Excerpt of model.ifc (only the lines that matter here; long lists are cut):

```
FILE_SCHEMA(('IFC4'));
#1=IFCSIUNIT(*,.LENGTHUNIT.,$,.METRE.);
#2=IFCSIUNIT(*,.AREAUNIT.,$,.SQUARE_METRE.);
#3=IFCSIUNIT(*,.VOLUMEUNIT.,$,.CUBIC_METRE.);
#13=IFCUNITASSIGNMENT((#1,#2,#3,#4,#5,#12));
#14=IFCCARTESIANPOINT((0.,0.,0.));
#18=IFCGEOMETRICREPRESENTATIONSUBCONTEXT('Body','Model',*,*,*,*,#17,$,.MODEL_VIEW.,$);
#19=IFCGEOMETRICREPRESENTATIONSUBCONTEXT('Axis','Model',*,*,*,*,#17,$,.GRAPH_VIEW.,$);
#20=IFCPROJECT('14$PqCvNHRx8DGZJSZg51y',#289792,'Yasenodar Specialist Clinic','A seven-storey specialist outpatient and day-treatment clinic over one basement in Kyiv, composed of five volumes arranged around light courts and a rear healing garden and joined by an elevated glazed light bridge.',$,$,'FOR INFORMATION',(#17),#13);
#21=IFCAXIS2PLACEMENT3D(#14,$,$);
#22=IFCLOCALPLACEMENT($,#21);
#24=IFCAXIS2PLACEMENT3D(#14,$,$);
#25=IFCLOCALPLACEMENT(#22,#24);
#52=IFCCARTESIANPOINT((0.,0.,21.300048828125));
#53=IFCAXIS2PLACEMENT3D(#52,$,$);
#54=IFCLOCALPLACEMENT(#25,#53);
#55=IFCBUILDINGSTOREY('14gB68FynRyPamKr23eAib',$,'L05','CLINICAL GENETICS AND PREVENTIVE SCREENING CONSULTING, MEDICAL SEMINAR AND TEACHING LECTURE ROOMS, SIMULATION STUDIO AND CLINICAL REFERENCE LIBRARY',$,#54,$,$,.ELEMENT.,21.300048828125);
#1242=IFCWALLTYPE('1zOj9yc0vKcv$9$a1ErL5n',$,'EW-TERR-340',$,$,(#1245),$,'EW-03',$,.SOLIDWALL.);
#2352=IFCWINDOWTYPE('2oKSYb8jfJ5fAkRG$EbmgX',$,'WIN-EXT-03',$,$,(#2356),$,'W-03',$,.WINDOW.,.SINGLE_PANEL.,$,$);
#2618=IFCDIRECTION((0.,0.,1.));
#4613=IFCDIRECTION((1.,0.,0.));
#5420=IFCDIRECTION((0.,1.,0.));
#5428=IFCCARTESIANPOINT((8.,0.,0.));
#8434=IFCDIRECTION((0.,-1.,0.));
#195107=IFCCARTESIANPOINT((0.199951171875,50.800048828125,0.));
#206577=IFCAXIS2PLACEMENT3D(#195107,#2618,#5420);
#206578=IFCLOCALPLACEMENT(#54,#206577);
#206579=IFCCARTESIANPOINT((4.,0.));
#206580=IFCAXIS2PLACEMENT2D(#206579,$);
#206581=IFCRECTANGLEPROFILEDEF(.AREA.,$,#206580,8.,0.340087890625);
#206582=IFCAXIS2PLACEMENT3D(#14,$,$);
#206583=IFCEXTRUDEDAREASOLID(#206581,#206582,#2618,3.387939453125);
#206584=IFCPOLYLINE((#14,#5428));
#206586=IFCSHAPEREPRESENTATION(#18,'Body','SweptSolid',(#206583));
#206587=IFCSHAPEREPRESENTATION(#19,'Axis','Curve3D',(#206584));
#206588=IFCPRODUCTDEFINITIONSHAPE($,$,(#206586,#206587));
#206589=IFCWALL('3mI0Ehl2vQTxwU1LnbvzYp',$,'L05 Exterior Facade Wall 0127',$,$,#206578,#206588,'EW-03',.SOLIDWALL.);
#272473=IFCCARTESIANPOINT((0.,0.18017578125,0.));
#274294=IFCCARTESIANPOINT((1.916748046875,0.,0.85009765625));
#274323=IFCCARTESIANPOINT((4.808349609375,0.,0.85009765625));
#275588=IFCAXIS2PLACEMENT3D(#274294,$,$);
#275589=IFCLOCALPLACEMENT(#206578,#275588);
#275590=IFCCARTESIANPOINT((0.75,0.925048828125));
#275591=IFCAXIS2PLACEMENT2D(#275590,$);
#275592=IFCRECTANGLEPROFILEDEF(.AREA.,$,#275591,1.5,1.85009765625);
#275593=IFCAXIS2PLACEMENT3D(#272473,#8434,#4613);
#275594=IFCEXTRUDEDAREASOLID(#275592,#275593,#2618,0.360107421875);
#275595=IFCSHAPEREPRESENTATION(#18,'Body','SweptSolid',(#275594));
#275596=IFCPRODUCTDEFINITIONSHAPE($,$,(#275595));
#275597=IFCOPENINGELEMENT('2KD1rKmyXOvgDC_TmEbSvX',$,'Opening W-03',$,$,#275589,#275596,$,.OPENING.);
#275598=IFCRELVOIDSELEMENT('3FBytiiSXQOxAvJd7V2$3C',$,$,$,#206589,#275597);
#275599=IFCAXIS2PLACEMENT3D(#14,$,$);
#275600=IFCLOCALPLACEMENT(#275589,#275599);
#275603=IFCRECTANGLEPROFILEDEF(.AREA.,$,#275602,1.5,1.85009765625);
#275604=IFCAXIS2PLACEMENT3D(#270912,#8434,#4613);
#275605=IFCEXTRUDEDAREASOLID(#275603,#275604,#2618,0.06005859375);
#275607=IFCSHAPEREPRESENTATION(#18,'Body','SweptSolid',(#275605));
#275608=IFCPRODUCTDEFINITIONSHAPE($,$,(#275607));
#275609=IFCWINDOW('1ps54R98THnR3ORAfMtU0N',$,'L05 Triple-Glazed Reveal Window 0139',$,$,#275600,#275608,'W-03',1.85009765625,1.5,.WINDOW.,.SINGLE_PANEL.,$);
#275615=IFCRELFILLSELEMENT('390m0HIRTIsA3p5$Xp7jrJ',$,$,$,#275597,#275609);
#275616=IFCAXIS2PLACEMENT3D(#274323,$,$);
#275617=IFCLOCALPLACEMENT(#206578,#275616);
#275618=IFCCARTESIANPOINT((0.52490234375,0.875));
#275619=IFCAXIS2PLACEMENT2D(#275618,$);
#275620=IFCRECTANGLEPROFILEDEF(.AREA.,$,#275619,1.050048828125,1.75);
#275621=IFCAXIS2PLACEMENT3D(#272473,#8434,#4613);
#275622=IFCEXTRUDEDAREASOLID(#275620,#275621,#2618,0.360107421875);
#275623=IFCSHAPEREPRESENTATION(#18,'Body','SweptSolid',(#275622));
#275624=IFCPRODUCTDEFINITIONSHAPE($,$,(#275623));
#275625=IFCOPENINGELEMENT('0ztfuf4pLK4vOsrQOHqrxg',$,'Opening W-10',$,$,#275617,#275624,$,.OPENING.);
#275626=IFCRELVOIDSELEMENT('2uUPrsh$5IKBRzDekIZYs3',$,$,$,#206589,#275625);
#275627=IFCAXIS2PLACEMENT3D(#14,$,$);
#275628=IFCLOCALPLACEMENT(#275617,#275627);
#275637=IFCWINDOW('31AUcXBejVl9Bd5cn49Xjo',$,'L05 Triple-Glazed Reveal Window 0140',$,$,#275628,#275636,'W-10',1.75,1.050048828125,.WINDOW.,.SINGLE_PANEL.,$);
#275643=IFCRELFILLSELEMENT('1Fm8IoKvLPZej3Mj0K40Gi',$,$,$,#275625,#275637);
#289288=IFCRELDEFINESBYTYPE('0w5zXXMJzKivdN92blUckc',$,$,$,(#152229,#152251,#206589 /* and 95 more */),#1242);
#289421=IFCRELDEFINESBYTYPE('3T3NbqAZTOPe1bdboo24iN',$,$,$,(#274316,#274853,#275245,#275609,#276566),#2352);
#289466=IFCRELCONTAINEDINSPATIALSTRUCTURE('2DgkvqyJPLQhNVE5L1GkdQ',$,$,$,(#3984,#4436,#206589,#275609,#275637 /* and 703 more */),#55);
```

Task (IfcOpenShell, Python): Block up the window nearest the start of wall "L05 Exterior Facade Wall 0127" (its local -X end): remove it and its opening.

```python
import ifcopenshell
import ifcopenshell.api.feature
import ifcopenshell.api.root
import ifcopenshell.geom
import ifcopenshell.util.shape

model = ifcopenshell.open("model.ifc")
settings = ifcopenshell.geom.settings()


def volume(element):
    """Net volume in cubic metres, openings subtracted."""
    shape = ifcopenshell.geom.create_shape(settings, element)
    return ifcopenshell.util.shape.get_volume(shape.geometry)


window = model.by_id(275609)
opening = window.FillsVoids[0].RelatingOpeningElement
wall = opening.VoidsElements[0].RelatingBuildingElement
before = volume(wall)

ifcopenshell.api.root.remove_product(model, product=window)
ifcopenshell.api.feature.remove_feature(model, feature=opening)

after = volume(wall)

print(f"wall volume {before:.3f} -> {after:.3f} m3")

model.write("model_rev.ifc")
```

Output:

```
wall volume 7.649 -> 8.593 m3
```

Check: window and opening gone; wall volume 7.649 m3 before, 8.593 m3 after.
